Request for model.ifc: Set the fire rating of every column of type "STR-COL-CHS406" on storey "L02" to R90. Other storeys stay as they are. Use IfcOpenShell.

First a look at what the model holds.

```python
import ifcopenshell
import ifcopenshell.util.element

model = ifcopenshell.open("model.ifc")
print(model.schema)
storey = next(s for s in model.by_type("IfcBuildingStorey") if s.Name == "L02")
columns = [e for e in ifcopenshell.util.element.get_decomposition(storey) if e.is_a("IfcColumn")]
seen = {}
for e in columns:
    element_type = ifcopenshell.util.element.get_type(e)
    key = (element_type.Name if element_type != e and element_type else None, ifcopenshell.util.element.get_pset(e, "Pset_ColumnCommon", "FireRating"))
    seen[key] = seen.get(key, 0) + 1
for (name, value), count in sorted(seen.items(), key=str):
    print(count, "x", name, "|", value)
```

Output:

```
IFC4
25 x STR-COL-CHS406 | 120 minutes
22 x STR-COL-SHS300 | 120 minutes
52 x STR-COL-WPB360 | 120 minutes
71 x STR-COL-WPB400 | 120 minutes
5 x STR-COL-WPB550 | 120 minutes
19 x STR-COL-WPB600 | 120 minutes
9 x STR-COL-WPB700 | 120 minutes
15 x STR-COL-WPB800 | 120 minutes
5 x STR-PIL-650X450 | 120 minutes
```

```python
import ifcopenshell
import ifcopenshell.api.pset
import ifcopenshell.util.element

model = ifcopenshell.open("model.ifc")

storey = next(s for s in model.by_type("IfcBuildingStorey") if s.Name == "L02")
columns = [e for e in ifcopenshell.util.element.get_decomposition(storey) if e.is_a("IfcColumn")]

count = 0
for e in columns:
    element_type = ifcopenshell.util.element.get_type(e)
    if element_type in (None, e) or element_type.Name != "STR-COL-CHS406":
        continue
    # add_pset returns the element's existing set when there is one.
    pset = ifcopenshell.api.pset.add_pset(model, product=e, name="Pset_ColumnCommon")
    ifcopenshell.api.pset.edit_pset(model, pset=pset, properties={"FireRating": "R90"})
    count += 1

print(count, "columns updated")

model.write("model_v2.ifc")
```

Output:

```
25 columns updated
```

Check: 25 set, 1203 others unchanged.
